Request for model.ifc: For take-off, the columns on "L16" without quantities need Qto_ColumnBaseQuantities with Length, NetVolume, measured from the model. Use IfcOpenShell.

First a look at what the model holds.

```python
import ifcopenshell
import ifcopenshell.util.element
import ifcopenshell.util.unit

model = ifcopenshell.open("model.ifc")
print(model.schema)
for unit_type in ("LENGTHUNIT", "AREAUNIT", "VOLUMEUNIT"):
    print(unit_type, ifcopenshell.util.unit.calculate_unit_scale(model, unit_type))
storey = next(s for s in model.by_type("IfcBuildingStorey") if s.Name == "L16")
columns = [e for e in ifcopenshell.util.element.get_decomposition(storey) if e.is_a("IfcColumn")]
for e in sorted(columns, key=lambda e: e.id()):
    print(e.id(), e.is_a(), e.Name, list(ifcopenshell.util.element.get_psets(e, qtos_only=True)), sep=" | ")
```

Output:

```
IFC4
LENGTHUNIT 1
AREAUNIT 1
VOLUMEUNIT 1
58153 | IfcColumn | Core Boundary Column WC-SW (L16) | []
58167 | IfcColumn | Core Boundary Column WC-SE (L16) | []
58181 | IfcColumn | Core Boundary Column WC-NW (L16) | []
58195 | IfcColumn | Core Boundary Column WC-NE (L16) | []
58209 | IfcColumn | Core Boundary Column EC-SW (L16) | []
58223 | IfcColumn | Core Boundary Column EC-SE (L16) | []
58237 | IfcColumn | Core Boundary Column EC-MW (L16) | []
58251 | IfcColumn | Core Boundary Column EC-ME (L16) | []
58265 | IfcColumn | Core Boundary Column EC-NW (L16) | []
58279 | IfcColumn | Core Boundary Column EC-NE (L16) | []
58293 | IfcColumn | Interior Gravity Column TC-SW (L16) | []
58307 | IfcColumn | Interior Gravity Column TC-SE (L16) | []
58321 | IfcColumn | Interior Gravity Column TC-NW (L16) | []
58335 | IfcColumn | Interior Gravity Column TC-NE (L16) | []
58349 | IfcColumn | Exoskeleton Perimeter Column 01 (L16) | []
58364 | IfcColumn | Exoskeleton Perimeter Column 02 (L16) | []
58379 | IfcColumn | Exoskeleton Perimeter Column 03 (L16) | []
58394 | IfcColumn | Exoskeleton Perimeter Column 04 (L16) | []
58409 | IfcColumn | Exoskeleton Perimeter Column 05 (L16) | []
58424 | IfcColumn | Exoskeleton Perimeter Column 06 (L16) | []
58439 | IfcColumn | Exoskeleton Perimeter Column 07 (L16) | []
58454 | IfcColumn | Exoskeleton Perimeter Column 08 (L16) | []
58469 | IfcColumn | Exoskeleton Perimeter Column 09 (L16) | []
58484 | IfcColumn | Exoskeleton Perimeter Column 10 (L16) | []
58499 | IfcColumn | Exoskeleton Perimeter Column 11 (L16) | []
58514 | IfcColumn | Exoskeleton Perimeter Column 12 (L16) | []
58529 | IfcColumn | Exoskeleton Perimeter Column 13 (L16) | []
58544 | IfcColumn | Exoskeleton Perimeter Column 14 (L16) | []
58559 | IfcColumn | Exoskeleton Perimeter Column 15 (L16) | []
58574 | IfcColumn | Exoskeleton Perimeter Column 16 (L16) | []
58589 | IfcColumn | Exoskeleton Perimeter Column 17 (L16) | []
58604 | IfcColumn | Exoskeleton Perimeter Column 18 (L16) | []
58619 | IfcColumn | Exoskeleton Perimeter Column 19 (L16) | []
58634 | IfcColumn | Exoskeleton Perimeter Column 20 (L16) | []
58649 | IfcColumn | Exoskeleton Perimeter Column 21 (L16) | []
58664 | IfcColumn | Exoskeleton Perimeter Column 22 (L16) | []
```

```python
import ifcopenshell
import ifcopenshell.api.pset
import ifcopenshell.geom
import ifcopenshell.util.element
import ifcopenshell.util.shape
import ifcopenshell.util.unit

model = ifcopenshell.open("model.ifc")
unit_scale = ifcopenshell.util.unit.calculate_unit_scale(model)
volume_scale = ifcopenshell.util.unit.calculate_unit_scale(model, "VOLUMEUNIT")
settings = ifcopenshell.geom.settings()

storey = next(s for s in model.by_type("IfcBuildingStorey") if s.Name == "L16")
columns = [e for e in ifcopenshell.util.element.get_decomposition(storey) if e.is_a("IfcColumn")]

for e in sorted(columns, key=lambda e: e.id()):
    if ifcopenshell.util.element.get_psets(e, qtos_only=True, should_inherit=False):
        continue
    # Geometry comes back in metres, in the element's own axes.
    shape = ifcopenshell.geom.create_shape(settings, e)
    values = {
        "Length": ifcopenshell.util.shape.get_z(shape.geometry) / unit_scale,
        "NetVolume": ifcopenshell.util.shape.get_volume(shape.geometry) / volume_scale,
    }
    qto = ifcopenshell.api.pset.add_qto(model, product=e, name="Qto_ColumnBaseQuantities")
    ifcopenshell.api.pset.edit_qto(model, qto=qto, properties=values)
    print(e.id(), {k: round(v, 3) for k, v in values.items()})

model.write("model-out.ifc")
```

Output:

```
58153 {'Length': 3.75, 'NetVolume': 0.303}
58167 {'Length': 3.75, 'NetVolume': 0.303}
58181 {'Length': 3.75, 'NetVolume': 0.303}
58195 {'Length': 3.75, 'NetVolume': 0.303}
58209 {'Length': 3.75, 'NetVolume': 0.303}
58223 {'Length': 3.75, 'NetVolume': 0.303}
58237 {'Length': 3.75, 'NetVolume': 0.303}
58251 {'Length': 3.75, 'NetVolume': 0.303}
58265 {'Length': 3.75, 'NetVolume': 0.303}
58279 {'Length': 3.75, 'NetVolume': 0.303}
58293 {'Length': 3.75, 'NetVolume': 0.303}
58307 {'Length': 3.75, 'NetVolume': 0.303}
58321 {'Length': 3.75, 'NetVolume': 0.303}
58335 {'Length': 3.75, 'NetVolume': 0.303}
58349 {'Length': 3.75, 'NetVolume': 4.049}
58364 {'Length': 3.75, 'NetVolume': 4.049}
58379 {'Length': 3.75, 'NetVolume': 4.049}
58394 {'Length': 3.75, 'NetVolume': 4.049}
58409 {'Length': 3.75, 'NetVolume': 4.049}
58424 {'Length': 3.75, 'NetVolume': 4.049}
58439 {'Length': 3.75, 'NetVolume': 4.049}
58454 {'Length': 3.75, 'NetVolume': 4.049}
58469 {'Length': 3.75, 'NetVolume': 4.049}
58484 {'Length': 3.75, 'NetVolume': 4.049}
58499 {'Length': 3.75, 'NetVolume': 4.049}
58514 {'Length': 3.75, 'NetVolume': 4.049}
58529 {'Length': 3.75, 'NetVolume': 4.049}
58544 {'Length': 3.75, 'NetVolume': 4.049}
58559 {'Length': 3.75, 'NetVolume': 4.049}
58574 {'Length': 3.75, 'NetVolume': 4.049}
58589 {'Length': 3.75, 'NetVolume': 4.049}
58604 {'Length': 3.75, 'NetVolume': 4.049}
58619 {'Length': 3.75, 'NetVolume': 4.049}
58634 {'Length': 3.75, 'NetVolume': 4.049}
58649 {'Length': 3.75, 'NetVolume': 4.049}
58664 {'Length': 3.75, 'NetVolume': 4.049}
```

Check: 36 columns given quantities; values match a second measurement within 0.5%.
